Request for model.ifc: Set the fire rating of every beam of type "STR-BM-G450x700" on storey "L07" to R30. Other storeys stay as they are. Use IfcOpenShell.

First a look at what the model holds.

```python
import ifcopenshell
import ifcopenshell.util.element

model = ifcopenshell.open("model.ifc")
print(model.schema)
storey = next(s for s in model.by_type("IfcBuildingStorey") if s.Name == "L07")
beams = [e for e in ifcopenshell.util.element.get_decomposition(storey) if e.is_a("IfcBeam")]
seen = {}
for e in beams:
    element_type = ifcopenshell.util.element.get_type(e)
    key = (element_type.Name if element_type != e and element_type else None, ifcopenshell.util.element.get_pset(e, "Pset_BeamCommon", "FireRating"))
    seen[key] = seen.get(key, 0) + 1
for (name, value), count in sorted(seen.items(), key=str):
    print(count, "x", name, "|", value)
```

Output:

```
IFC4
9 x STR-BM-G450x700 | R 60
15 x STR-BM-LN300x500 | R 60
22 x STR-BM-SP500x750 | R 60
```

```python
import ifcopenshell
import ifcopenshell.api.pset
import ifcopenshell.util.element

model = ifcopenshell.open("model.ifc")

storey = next(s for s in model.by_type("IfcBuildingStorey") if s.Name == "L07")
beams = [e for e in ifcopenshell.util.element.get_decomposition(storey) if e.is_a("IfcBeam")]

count = 0
for e in beams:
    element_type = ifcopenshell.util.element.get_type(e)
    if element_type in (None, e) or element_type.Name != "STR-BM-G450x700":
        continue
    # add_pset returns the element's existing set when there is one.
    pset = ifcopenshell.api.pset.add_pset(model, product=e, name="Pset_BeamCommon")
    ifcopenshell.api.pset.edit_pset(model, pset=pset, properties={"FireRating": "R30"})
    count += 1

print(count, "beams updated")

model.write("model_v2.ifc")
```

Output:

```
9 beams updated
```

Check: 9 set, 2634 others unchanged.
